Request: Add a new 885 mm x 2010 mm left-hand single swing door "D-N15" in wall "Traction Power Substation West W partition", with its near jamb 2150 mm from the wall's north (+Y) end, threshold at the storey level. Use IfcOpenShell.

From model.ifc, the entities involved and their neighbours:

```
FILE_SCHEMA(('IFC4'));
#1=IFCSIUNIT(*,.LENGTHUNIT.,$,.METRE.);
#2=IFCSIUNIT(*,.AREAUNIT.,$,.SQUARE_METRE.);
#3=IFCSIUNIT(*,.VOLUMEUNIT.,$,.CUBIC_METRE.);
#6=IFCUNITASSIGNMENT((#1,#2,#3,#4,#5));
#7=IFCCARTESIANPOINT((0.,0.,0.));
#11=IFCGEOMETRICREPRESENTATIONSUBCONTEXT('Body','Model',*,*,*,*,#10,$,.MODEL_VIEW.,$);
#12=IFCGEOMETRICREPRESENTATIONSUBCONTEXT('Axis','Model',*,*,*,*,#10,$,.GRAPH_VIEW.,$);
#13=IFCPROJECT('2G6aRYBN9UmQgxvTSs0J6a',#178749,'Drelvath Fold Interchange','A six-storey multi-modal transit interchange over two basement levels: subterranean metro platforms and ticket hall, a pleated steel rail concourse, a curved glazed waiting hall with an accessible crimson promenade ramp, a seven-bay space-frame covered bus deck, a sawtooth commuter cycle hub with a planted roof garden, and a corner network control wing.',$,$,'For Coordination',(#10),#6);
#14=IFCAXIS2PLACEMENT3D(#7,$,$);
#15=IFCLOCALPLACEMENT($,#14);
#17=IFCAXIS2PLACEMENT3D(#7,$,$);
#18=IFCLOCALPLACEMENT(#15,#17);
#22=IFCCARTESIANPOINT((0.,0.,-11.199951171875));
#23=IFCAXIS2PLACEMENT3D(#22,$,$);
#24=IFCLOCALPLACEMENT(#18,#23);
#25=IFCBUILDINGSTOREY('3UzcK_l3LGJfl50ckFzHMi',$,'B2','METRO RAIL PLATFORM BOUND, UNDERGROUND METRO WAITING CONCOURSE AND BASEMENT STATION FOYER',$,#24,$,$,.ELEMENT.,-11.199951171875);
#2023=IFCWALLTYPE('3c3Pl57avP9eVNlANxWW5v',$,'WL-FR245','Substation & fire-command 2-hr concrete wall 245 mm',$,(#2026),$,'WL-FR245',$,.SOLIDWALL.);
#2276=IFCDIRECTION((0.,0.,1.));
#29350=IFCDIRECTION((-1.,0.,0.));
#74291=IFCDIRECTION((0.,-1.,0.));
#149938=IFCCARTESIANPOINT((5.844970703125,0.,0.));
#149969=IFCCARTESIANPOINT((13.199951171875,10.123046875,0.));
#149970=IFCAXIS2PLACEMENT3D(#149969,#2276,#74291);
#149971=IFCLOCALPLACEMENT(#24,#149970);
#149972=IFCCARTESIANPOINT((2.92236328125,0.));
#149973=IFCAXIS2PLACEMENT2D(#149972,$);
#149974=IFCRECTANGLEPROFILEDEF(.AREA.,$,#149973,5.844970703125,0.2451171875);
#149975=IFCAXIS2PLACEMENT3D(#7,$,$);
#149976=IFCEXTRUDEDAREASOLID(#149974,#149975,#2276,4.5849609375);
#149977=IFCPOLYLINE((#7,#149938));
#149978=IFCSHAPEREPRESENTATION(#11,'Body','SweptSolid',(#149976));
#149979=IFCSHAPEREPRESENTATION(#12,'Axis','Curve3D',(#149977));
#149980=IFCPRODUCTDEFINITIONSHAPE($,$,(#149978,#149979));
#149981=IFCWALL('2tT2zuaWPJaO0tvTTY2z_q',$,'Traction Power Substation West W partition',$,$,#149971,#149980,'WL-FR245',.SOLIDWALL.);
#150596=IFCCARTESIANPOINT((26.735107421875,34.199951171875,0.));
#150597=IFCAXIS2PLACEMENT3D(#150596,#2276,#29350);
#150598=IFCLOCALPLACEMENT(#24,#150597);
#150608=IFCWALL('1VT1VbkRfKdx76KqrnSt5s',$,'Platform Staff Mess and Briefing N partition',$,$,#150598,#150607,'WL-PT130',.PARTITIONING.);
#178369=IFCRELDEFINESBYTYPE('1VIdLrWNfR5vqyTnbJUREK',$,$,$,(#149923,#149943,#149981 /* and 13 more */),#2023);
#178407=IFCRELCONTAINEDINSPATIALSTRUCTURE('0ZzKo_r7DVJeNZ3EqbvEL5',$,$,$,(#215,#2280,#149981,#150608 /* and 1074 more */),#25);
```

```python
import numpy as np
import ifcopenshell
import ifcopenshell.api.feature
import ifcopenshell.api.geometry
import ifcopenshell.api.root
import ifcopenshell.api.spatial
import ifcopenshell.geom
import ifcopenshell.util.element
import ifcopenshell.util.placement
import ifcopenshell.util.representation
import ifcopenshell.util.shape
import ifcopenshell.util.unit

model = ifcopenshell.open("model.ifc")
unit_scale = ifcopenshell.util.unit.calculate_unit_scale(model)
settings = ifcopenshell.geom.settings()


def volume(element):
    """Net volume in cubic metres, openings subtracted."""
    shape = ifcopenshell.geom.create_shape(settings, element)
    return ifcopenshell.util.shape.get_volume(shape.geometry)


wall = model.by_guid("2tT2zuaWPJaO0tvTTY2z_q")
storey = ifcopenshell.util.element.get_container(wall, ifc_class="IfcBuildingStorey")
context = ifcopenshell.util.representation.get_context(model, "Model", "Body", "MODEL_VIEW")
before = volume(wall)

width, height, from_end, sill = 0.885, 2.01, 2.15, 0.0  # metres

# The wall runs along its own X axis, and the end named is its -X end.
wall_shape = ifcopenshell.geom.create_shape(settings, wall)
x, y, z = ifcopenshell.util.shape.get_vertices(wall_shape.geometry).T
start = x.min() + from_end
face, thickness = float(y.min()), float(y.max() - y.min())
wall_matrix = ifcopenshell.util.placement.get_local_placement(wall.ObjectPlacement)
level = ifcopenshell.util.placement.get_local_placement(storey.ObjectPlacement)[2, 3]


def in_wall(x, y):
    """Placement at x, y metres in the wall's axes, at sill height."""
    matrix = wall_matrix.copy()
    matrix[:, 3] = wall_matrix @ np.array([x / unit_scale, y / unit_scale, 0.0, 1.0])
    matrix[2, 3] = level + sill / unit_scale
    return matrix


# Opening: a box that overshoots both wall faces by 50 mm.
opening = ifcopenshell.api.root.create_entity(model, ifc_class="IfcOpeningElement", predefined_type="OPENING")
box = ifcopenshell.api.geometry.add_wall_representation(
    model, context=context, length=width, height=height, thickness=thickness + 0.1
)
ifcopenshell.api.geometry.assign_representation(model, product=opening, representation=box)
ifcopenshell.api.geometry.edit_object_placement(model, product=opening, matrix=in_wall(start, face - 0.05), is_si=False)
ifcopenshell.api.feature.add_feature(model, feature=opening, element=wall)

door = ifcopenshell.api.root.create_entity(model, ifc_class="IfcDoor", name="D-N15", predefined_type="DOOR")
door.OverallWidth, door.OverallHeight = width / unit_scale, height / unit_scale
door.OperationType = "SINGLE_SWING_LEFT"
body = ifcopenshell.api.geometry.add_door_representation(
    model,
    context=context,
    overall_width=door.OverallWidth,
    overall_height=door.OverallHeight,
    operation_type="SINGLE_SWING_LEFT",
    lining_properties={"LiningDepth": thickness / unit_scale, "ThresholdDepth": thickness / unit_scale},
)
ifcopenshell.api.geometry.assign_representation(model, product=door, representation=body)
ifcopenshell.api.spatial.assign_container(model, products=[door], relating_structure=storey)
ifcopenshell.api.feature.add_filling(model, opening=opening, element=door)

# The lining spans the wall, so the door starts at the wall face.
ifcopenshell.api.geometry.edit_object_placement(model, product=door, matrix=in_wall(start, face), is_si=False)

after = volume(wall)

print(f"wall volume {before:.3f} -> {after:.3f} m3")

model.write("model_edited.ifc")
```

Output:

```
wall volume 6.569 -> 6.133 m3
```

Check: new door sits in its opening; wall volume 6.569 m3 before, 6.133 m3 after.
